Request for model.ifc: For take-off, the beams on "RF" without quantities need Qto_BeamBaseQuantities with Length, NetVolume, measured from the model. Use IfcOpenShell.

First a look at what the model holds.

```python
import ifcopenshell
import ifcopenshell.util.element
import ifcopenshell.util.unit

model = ifcopenshell.open("model.ifc")
print(model.schema)
for unit_type in ("LENGTHUNIT", "AREAUNIT", "VOLUMEUNIT"):
    print(unit_type, ifcopenshell.util.unit.calculate_unit_scale(model, unit_type))
storey = next(s for s in model.by_type("IfcBuildingStorey") if s.Name == "RF")
beams = [e for e in ifcopenshell.util.element.get_decomposition(storey) if e.is_a("IfcBeam")]
for e in sorted(beams, key=lambda e: e.id()):
    print(e.id(), e.is_a(), e.Name, list(ifcopenshell.util.element.get_psets(e, qtos_only=True)), sep=" | ")
```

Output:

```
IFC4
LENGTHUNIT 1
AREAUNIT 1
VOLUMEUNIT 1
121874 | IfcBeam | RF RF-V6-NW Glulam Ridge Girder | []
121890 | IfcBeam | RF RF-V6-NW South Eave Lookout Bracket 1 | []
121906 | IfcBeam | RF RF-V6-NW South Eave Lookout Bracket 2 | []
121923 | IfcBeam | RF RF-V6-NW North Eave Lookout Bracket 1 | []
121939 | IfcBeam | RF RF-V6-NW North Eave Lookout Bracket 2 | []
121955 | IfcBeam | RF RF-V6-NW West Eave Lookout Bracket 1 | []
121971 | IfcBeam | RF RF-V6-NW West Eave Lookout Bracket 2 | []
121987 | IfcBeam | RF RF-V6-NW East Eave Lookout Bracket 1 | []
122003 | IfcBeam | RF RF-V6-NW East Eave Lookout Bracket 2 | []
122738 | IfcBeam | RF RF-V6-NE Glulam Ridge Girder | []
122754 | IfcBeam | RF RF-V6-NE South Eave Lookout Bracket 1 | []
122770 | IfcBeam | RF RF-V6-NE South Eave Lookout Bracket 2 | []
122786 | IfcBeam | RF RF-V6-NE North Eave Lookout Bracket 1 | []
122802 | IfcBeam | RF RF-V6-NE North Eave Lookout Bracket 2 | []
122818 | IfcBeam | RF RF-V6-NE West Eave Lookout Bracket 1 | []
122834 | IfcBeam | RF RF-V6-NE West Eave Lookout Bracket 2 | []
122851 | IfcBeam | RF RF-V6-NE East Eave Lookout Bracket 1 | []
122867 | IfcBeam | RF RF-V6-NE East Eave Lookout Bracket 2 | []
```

```python
import ifcopenshell
import ifcopenshell.api.pset
import ifcopenshell.geom
import ifcopenshell.util.element
import ifcopenshell.util.shape
import ifcopenshell.util.unit

model = ifcopenshell.open("model.ifc")
unit_scale = ifcopenshell.util.unit.calculate_unit_scale(model)
volume_scale = ifcopenshell.util.unit.calculate_unit_scale(model, "VOLUMEUNIT")
settings = ifcopenshell.geom.settings()

storey = next(s for s in model.by_type("IfcBuildingStorey") if s.Name == "RF")
beams = [e for e in ifcopenshell.util.element.get_decomposition(storey) if e.is_a("IfcBeam")]

for e in sorted(beams, key=lambda e: e.id()):
    if ifcopenshell.util.element.get_psets(e, qtos_only=True, should_inherit=False):
        continue
    # Geometry comes back in metres, in the element's own axes.
    shape = ifcopenshell.geom.create_shape(settings, e)
    values = {
        "Length": ifcopenshell.util.shape.get_max_xyz(shape.geometry) / unit_scale,
        "NetVolume": ifcopenshell.util.shape.get_volume(shape.geometry) / volume_scale,
    }
    qto = ifcopenshell.api.pset.add_qto(model, product=e, name="Qto_BeamBaseQuantities")
    ifcopenshell.api.pset.edit_qto(model, qto=qto, properties=values)
    print(e.id(), {k: round(v, 3) for k, v in values.items()})

model.write("model_edited.ifc")
```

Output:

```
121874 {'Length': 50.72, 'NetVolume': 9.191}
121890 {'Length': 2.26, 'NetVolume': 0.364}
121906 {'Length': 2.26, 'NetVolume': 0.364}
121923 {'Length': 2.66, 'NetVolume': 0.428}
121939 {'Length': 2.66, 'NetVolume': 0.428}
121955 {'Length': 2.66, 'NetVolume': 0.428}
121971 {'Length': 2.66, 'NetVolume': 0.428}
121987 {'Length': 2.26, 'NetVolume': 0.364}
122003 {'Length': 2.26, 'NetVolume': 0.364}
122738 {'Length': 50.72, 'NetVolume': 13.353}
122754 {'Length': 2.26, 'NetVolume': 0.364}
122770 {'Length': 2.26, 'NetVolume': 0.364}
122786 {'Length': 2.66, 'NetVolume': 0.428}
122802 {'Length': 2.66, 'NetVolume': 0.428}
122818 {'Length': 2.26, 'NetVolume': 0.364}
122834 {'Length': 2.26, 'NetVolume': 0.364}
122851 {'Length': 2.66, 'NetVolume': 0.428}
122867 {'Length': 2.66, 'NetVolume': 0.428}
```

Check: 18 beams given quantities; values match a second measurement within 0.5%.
